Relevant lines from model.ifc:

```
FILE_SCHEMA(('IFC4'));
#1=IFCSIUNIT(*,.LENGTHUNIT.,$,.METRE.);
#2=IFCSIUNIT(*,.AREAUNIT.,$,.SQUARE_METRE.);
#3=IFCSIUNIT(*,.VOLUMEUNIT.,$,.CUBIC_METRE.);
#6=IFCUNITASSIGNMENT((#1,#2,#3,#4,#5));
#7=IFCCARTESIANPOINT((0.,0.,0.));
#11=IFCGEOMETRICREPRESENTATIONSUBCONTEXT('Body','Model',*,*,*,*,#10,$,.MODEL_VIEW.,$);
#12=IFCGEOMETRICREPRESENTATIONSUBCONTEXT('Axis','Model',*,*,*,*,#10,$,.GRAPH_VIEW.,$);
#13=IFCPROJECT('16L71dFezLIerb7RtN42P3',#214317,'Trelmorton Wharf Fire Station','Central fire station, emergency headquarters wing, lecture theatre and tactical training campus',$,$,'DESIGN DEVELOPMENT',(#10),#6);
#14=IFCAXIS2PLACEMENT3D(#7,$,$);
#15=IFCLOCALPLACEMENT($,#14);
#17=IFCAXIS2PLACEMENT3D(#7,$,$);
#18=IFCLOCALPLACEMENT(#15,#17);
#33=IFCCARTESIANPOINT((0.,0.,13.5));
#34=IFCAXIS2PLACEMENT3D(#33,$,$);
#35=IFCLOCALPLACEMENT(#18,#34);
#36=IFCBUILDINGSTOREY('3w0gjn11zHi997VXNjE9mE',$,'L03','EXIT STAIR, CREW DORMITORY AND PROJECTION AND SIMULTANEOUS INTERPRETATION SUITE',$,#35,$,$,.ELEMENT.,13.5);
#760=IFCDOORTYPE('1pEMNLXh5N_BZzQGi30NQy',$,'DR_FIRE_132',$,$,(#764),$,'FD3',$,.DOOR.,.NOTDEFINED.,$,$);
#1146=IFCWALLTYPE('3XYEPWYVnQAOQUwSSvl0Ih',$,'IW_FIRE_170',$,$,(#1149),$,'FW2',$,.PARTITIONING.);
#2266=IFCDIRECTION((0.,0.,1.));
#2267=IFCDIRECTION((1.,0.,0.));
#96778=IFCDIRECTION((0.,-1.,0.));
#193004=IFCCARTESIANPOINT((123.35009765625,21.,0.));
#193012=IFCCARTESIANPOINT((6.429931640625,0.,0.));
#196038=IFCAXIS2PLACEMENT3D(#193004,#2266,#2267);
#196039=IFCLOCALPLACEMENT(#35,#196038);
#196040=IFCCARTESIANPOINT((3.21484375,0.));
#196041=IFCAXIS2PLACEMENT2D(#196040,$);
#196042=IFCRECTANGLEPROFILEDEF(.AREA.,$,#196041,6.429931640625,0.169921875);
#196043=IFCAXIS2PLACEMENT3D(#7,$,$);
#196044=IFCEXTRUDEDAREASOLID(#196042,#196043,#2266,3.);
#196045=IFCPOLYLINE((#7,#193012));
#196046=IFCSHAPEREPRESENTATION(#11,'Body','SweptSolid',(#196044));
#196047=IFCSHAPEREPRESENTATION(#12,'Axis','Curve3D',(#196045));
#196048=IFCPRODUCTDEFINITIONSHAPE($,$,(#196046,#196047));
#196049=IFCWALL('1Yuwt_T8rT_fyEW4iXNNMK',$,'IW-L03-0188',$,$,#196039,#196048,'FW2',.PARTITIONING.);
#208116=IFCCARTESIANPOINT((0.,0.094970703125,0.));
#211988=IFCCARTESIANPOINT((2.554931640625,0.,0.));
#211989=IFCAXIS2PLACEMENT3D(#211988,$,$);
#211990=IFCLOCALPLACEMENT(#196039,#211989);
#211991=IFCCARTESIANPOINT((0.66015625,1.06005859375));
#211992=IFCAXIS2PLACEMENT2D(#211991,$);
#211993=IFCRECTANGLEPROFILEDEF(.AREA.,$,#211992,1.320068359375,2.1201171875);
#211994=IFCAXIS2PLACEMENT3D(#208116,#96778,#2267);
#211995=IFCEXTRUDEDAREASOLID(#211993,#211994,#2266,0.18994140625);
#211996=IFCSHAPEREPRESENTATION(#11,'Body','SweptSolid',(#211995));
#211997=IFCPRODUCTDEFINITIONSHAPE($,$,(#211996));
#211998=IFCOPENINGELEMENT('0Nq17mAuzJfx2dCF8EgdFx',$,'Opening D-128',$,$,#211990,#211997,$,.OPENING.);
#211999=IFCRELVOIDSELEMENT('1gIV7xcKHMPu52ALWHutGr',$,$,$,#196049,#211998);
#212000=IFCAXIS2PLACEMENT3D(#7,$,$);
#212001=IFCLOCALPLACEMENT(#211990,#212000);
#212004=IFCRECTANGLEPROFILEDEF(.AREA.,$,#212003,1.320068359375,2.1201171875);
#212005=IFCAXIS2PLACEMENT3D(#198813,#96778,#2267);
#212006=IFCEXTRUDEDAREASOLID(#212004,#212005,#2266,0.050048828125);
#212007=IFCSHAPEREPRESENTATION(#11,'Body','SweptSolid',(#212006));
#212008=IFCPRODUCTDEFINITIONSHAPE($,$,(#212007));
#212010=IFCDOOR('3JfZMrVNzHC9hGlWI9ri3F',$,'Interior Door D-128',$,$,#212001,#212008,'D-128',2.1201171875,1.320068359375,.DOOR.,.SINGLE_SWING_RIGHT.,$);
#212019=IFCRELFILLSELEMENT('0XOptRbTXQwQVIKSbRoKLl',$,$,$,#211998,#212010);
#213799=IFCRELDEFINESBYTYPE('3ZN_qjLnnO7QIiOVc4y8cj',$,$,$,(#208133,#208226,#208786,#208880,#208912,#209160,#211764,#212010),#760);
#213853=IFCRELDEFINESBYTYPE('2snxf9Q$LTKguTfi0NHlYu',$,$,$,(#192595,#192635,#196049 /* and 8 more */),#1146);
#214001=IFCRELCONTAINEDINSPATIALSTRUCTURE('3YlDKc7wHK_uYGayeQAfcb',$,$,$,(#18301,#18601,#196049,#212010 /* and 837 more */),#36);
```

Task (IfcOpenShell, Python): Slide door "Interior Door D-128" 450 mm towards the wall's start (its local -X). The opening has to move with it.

```python
import ifcopenshell
import ifcopenshell.api.geometry
import ifcopenshell.util.placement
import ifcopenshell.util.unit

model = ifcopenshell.open("model.ifc")
unit_scale = ifcopenshell.util.unit.calculate_unit_scale(model)

door = model.by_guid("3JfZMrVNzHC9hGlWI9ri3F")
opening = door.FillsVoids[0].RelatingOpeningElement
wall = opening.VoidsElements[0].RelatingBuildingElement

wall_matrix = ifcopenshell.util.placement.get_local_placement(wall.ObjectPlacement)
shift = wall_matrix[:3, 0] * -0.45 / unit_scale
before = ifcopenshell.util.placement.get_local_placement(door.ObjectPlacement)[:3, 3].copy()

# The door is placed relative to its opening, so it follows when the opening moves.
matrix = ifcopenshell.util.placement.get_local_placement(opening.ObjectPlacement)
matrix[:3, 3] += shift
ifcopenshell.api.geometry.edit_object_placement(
    model, product=opening, matrix=matrix, is_si=False, should_transform_children=True
)

after = ifcopenshell.util.placement.get_local_placement(door.ObjectPlacement)[:3, 3]
print("door moved by", (after - before).round(3) + 0.0)

model.write("model-out.ifc")
```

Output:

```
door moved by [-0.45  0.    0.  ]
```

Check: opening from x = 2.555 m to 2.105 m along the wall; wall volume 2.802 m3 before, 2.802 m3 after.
